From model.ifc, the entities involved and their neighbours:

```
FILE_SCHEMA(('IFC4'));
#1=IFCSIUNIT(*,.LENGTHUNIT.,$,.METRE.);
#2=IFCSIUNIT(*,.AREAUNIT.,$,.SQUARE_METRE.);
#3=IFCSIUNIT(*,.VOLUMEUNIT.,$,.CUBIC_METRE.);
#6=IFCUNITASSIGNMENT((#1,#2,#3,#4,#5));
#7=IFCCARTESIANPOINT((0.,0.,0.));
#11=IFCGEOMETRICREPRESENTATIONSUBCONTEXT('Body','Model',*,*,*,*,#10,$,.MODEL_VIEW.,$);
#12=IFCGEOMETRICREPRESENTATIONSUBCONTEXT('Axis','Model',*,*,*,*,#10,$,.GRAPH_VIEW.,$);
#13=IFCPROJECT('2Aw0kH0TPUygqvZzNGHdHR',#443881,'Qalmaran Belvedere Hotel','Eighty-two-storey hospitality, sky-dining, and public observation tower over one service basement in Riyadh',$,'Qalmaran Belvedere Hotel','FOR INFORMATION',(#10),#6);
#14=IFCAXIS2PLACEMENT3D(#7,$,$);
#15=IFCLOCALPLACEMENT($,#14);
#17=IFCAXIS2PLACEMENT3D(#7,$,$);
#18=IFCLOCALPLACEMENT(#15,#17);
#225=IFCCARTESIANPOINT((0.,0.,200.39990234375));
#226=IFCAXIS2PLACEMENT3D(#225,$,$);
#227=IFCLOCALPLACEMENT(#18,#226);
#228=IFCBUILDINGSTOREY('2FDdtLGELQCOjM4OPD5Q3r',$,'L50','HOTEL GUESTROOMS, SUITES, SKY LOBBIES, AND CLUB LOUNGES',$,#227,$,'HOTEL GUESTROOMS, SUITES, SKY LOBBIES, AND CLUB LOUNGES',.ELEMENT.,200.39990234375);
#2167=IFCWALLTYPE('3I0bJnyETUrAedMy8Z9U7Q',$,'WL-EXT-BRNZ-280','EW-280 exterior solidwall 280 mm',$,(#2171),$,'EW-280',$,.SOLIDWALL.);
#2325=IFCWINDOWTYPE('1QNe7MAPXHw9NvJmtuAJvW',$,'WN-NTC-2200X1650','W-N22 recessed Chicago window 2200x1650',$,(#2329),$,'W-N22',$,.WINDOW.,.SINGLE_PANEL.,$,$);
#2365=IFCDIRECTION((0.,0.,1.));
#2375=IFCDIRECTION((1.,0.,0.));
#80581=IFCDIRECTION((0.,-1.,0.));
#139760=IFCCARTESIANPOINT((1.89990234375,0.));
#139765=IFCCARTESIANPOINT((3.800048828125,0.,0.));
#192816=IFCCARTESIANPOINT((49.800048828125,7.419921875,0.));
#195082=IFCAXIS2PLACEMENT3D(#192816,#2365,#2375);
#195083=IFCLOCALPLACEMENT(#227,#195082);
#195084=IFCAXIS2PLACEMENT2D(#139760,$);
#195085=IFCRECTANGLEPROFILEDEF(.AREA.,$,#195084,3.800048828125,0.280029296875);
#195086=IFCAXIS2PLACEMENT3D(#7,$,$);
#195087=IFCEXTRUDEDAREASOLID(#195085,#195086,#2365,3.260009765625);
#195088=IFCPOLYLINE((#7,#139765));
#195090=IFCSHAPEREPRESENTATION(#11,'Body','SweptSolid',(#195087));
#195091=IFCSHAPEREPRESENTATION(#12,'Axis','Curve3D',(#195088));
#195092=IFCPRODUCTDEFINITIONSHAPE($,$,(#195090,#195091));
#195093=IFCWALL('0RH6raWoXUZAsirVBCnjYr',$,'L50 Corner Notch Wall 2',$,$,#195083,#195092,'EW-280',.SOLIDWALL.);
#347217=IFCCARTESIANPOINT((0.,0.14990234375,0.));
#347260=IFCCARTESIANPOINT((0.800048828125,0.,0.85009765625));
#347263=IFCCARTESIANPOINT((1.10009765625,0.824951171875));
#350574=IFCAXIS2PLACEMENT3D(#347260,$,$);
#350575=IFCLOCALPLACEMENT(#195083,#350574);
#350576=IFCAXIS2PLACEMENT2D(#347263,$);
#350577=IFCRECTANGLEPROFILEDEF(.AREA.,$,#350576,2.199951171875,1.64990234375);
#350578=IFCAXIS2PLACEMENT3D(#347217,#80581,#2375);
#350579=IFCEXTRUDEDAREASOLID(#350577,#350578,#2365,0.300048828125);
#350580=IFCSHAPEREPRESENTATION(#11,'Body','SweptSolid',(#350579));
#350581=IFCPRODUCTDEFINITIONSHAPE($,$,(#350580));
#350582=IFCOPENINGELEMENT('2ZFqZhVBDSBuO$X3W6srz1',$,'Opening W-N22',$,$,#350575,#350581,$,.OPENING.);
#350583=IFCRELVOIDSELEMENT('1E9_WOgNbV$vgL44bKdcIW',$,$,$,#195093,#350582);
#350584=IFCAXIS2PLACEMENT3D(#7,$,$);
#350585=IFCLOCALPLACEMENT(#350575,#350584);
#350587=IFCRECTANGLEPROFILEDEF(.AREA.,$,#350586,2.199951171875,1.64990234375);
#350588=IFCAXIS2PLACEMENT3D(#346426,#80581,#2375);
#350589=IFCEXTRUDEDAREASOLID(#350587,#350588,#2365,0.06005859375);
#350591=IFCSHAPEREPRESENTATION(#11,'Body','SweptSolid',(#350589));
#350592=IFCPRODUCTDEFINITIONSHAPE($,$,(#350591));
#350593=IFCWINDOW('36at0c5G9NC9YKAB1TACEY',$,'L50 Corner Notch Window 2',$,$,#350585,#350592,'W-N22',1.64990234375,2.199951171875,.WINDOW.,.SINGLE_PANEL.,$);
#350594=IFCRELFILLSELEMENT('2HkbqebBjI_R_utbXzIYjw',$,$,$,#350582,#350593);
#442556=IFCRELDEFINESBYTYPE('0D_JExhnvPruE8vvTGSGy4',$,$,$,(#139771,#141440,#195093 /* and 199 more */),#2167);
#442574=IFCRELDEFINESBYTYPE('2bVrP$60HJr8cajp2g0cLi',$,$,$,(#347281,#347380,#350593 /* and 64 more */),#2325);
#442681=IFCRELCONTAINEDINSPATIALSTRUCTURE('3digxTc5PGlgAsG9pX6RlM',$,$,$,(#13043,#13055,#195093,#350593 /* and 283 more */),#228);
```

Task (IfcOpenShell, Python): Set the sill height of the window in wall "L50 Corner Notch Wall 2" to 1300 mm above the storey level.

```python
import numpy as np
import ifcopenshell
import ifcopenshell.api.geometry
import ifcopenshell.geom
import ifcopenshell.util.element
import ifcopenshell.util.placement
import ifcopenshell.util.shape
import ifcopenshell.util.unit

model = ifcopenshell.open("model.ifc")
unit_scale = ifcopenshell.util.unit.calculate_unit_scale(model)

window = model.by_guid("36at0c5G9NC9YKAB1TACEY")
opening = window.FillsVoids[0].RelatingOpeningElement
storey = ifcopenshell.util.element.get_container(window, ifc_class="IfcBuildingStorey")
level = ifcopenshell.util.placement.get_local_placement(storey.ObjectPlacement)[2, 3]

# The opening's origin need not be at the sill, so measure its lowest point.
shape = ifcopenshell.geom.create_shape(ifcopenshell.geom.settings(), opening)
bottom = ifcopenshell.util.shape.get_shape_bottom_elevation(shape, shape.geometry) / unit_scale
dz = level + 1.3 - bottom

shift = np.array([0.0, 0.0, dz])
# The window is placed relative to its opening, so it follows when the opening moves.
matrix = ifcopenshell.util.placement.get_local_placement(opening.ObjectPlacement)
matrix[:3, 3] += shift
ifcopenshell.api.geometry.edit_object_placement(
    model, product=opening, matrix=matrix, is_si=False, should_transform_children=True
)

print(f"moved by {dz * unit_scale:+.3f} m")

model.write("model-out.ifc")
```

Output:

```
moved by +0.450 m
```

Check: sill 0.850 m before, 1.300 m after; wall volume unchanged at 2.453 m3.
